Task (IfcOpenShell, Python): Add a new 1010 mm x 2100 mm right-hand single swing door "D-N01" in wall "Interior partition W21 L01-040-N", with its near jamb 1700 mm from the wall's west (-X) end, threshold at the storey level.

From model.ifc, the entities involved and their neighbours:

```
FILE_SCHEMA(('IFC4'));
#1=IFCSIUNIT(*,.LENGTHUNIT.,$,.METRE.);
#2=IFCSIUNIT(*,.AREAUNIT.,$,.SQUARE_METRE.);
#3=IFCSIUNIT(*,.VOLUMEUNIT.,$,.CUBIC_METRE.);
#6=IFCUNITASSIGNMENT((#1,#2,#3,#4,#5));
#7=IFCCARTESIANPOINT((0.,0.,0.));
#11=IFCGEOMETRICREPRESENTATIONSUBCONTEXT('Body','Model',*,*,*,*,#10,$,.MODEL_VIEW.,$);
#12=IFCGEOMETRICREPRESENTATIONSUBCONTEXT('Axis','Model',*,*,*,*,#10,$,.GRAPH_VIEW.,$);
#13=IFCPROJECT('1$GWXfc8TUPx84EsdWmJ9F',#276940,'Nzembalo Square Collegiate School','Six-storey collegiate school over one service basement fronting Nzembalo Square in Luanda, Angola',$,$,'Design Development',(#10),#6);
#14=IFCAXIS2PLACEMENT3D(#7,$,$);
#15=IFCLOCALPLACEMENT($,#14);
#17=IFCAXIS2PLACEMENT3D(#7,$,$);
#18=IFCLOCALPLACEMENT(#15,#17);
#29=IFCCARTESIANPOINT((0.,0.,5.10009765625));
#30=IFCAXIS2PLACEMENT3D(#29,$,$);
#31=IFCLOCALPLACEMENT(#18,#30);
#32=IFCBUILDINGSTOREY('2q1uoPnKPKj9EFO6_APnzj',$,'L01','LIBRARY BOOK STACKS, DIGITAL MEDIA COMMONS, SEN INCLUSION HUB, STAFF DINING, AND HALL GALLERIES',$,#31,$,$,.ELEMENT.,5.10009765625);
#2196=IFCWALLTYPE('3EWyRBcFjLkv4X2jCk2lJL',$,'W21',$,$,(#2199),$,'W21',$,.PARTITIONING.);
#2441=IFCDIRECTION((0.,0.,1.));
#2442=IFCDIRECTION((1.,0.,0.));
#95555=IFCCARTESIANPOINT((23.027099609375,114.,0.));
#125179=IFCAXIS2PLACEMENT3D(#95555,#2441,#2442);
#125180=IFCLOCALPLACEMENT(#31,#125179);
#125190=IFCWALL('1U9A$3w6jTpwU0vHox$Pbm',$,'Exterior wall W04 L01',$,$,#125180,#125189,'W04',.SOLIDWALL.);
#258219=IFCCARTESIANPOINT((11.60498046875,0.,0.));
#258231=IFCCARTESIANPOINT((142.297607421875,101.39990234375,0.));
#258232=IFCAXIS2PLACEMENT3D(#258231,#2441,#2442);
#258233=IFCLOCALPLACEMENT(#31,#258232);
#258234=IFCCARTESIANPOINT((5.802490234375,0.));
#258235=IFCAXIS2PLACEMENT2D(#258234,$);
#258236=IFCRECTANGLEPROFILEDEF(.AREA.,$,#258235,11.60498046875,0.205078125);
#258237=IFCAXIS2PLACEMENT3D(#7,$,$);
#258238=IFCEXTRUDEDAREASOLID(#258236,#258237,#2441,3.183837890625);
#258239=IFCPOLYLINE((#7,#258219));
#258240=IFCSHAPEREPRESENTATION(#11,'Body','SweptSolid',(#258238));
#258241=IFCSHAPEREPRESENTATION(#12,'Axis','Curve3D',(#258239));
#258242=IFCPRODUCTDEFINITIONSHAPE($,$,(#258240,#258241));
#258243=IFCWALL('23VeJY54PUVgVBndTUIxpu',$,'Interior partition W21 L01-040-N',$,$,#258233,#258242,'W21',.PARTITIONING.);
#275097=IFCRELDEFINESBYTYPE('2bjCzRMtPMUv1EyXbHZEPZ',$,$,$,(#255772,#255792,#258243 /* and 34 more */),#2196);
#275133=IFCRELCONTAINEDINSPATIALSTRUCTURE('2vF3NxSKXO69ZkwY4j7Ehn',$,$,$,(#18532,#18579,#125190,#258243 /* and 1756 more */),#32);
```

```python
import numpy as np
import ifcopenshell
import ifcopenshell.api.feature
import ifcopenshell.api.geometry
import ifcopenshell.api.root
import ifcopenshell.api.spatial
import ifcopenshell.geom
import ifcopenshell.util.element
import ifcopenshell.util.placement
import ifcopenshell.util.representation
import ifcopenshell.util.shape
import ifcopenshell.util.unit

model = ifcopenshell.open("model.ifc")
unit_scale = ifcopenshell.util.unit.calculate_unit_scale(model)
settings = ifcopenshell.geom.settings()


def volume(element):
    """Net volume in cubic metres, openings subtracted."""
    shape = ifcopenshell.geom.create_shape(settings, element)
    return ifcopenshell.util.shape.get_volume(shape.geometry)


wall = model.by_guid("23VeJY54PUVgVBndTUIxpu")
storey = ifcopenshell.util.element.get_container(wall, ifc_class="IfcBuildingStorey")
context = ifcopenshell.util.representation.get_context(model, "Model", "Body", "MODEL_VIEW")
before = volume(wall)

width, height, from_end, sill = 1.01, 2.1, 1.7, 0.0  # metres

# The wall runs along its own X axis, and the end named is its -X end.
wall_shape = ifcopenshell.geom.create_shape(settings, wall)
x, y, z = ifcopenshell.util.shape.get_vertices(wall_shape.geometry).T
start = x.min() + from_end
face, thickness = float(y.min()), float(y.max() - y.min())
wall_matrix = ifcopenshell.util.placement.get_local_placement(wall.ObjectPlacement)
level = ifcopenshell.util.placement.get_local_placement(storey.ObjectPlacement)[2, 3]


def in_wall(x, y):
    """Placement at x, y metres in the wall's axes, at sill height."""
    matrix = wall_matrix.copy()
    matrix[:, 3] = wall_matrix @ np.array([x / unit_scale, y / unit_scale, 0.0, 1.0])
    matrix[2, 3] = level + sill / unit_scale
    return matrix


# Opening: a box that overshoots both wall faces by 50 mm.
opening = ifcopenshell.api.root.create_entity(model, ifc_class="IfcOpeningElement", predefined_type="OPENING")
box = ifcopenshell.api.geometry.add_wall_representation(
    model, context=context, length=width, height=height, thickness=thickness + 0.1
)
ifcopenshell.api.geometry.assign_representation(model, product=opening, representation=box)
ifcopenshell.api.geometry.edit_object_placement(model, product=opening, matrix=in_wall(start, face - 0.05), is_si=False)
ifcopenshell.api.feature.add_feature(model, feature=opening, element=wall)

door = ifcopenshell.api.root.create_entity(model, ifc_class="IfcDoor", name="D-N01", predefined_type="DOOR")
door.OverallWidth, door.OverallHeight = width / unit_scale, height / unit_scale
door.OperationType = "SINGLE_SWING_RIGHT"
body = ifcopenshell.api.geometry.add_door_representation(
    model,
    context=context,
    overall_width=door.OverallWidth,
    overall_height=door.OverallHeight,
    operation_type="SINGLE_SWING_RIGHT",
    lining_properties={"LiningDepth": thickness / unit_scale, "ThresholdDepth": thickness / unit_scale},
)
ifcopenshell.api.geometry.assign_representation(model, product=door, representation=body)
ifcopenshell.api.spatial.assign_container(model, products=[door], relating_structure=storey)
ifcopenshell.api.feature.add_filling(model, opening=opening, element=door)

# The lining spans the wall, so the door starts at the wall face.
ifcopenshell.api.geometry.edit_object_placement(model, product=door, matrix=in_wall(start, face), is_si=False)

after = volume(wall)

print(f"wall volume {before:.3f} -> {after:.3f} m3")

model.write("model_v2.ifc")
```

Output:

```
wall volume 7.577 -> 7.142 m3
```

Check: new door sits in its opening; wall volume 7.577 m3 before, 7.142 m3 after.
